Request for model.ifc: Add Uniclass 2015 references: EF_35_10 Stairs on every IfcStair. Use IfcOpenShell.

First a look at what the model holds.

```python
import ifcopenshell

model = ifcopenshell.open("model.ifc")
print(model.schema)
print("classifications:", [c.Name for c in model.by_type("IfcClassification")])
for ifc_class in ("IfcDoor", "IfcRoof", "IfcStair", "IfcWall", "IfcWindow"):
    print(ifc_class, len(model.by_type(ifc_class)))
```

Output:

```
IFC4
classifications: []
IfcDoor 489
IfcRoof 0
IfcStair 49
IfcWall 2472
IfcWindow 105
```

```python
import ifcopenshell
import ifcopenshell.api.classification

model = ifcopenshell.open("model.ifc")

system = ifcopenshell.api.classification.add_classification(model, classification="Uniclass 2015")

codes = {
    "IfcStair": ("EF_35_10", "Stairs"),
}
for ifc_class, (code, name) in codes.items():
    products = model.by_type(ifc_class)
    ifcopenshell.api.classification.add_reference(
        model, products=products, classification=system, identification=code, name=name
    )
    print(code, len(products))

model.write("model_updated.ifc")
```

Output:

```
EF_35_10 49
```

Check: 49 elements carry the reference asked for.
